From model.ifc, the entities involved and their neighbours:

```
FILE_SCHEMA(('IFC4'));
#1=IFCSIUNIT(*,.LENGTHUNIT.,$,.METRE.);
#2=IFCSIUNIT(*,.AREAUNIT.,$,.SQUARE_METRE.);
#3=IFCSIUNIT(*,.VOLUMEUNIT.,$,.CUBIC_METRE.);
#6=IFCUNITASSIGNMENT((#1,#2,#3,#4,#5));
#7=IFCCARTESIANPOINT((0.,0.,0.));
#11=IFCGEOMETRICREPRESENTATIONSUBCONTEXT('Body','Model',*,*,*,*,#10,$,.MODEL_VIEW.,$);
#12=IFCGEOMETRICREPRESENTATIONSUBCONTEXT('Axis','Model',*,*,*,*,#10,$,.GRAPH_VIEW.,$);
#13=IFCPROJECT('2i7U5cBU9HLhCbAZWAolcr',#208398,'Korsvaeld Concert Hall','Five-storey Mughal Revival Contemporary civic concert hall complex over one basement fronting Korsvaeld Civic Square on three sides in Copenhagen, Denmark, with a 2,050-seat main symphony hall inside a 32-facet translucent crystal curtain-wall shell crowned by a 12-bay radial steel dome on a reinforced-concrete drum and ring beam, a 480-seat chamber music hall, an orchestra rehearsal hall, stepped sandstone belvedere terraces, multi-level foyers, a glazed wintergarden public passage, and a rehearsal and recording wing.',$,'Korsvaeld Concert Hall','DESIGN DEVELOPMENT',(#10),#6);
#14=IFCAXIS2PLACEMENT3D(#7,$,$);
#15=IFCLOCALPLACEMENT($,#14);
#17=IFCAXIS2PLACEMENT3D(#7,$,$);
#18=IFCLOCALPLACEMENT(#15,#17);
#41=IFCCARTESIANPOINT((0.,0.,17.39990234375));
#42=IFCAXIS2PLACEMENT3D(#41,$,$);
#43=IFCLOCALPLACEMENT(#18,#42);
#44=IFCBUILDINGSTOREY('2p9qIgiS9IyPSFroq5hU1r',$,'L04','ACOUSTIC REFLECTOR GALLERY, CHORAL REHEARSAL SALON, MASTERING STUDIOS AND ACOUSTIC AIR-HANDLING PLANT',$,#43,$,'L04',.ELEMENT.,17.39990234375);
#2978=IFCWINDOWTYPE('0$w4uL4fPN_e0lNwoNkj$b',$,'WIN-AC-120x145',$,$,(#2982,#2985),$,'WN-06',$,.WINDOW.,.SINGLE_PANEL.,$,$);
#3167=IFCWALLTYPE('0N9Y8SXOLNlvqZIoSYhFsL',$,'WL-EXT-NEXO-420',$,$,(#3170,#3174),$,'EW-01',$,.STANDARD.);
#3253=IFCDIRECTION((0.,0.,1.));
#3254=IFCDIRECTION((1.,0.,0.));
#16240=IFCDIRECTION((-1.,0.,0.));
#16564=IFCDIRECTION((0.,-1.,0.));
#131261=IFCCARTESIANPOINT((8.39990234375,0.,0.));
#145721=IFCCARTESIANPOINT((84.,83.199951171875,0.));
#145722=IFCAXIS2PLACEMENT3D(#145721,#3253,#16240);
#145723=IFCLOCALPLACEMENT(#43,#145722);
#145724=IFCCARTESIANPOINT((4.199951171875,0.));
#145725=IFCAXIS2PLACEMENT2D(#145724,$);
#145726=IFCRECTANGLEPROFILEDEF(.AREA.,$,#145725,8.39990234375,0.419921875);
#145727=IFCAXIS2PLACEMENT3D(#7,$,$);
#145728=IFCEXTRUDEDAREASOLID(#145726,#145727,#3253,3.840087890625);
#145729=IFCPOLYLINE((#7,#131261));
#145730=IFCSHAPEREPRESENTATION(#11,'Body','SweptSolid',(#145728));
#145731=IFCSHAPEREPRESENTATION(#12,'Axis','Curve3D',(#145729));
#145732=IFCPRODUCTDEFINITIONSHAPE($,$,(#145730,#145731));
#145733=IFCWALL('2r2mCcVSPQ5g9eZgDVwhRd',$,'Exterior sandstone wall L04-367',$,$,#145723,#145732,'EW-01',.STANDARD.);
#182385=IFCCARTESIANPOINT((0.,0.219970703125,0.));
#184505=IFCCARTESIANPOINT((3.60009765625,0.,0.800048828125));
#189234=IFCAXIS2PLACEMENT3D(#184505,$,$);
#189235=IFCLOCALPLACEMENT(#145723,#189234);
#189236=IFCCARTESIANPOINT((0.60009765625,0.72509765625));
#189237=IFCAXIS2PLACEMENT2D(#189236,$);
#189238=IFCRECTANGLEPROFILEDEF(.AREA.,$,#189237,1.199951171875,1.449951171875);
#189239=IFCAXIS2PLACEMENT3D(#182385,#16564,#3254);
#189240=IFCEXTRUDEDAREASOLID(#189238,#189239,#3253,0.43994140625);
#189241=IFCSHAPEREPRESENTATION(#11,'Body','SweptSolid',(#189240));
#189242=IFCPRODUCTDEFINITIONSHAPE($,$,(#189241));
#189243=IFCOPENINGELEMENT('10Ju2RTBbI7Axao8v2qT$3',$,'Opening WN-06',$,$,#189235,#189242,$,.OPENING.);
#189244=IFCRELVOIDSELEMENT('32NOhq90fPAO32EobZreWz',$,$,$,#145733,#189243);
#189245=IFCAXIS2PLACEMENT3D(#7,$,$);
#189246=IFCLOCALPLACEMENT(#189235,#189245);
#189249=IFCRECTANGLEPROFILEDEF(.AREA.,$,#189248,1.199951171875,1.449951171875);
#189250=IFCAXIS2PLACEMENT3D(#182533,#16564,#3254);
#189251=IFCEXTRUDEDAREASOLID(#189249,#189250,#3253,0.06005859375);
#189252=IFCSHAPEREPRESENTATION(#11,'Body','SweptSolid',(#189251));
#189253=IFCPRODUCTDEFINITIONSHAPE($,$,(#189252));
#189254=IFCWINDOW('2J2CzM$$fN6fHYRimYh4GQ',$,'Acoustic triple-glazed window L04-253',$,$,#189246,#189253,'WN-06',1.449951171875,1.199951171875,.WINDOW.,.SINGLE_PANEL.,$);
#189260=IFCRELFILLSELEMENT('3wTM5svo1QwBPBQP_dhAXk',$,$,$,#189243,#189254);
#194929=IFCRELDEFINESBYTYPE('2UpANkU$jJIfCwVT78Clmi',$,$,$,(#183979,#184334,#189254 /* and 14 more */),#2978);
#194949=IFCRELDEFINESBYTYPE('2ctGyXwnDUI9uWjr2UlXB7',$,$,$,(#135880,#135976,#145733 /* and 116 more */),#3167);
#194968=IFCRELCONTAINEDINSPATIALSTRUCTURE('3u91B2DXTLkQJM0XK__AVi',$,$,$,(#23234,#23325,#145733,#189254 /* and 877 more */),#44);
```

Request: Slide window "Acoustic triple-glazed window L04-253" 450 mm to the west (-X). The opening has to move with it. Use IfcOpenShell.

```python
import ifcopenshell
import ifcopenshell.api.geometry
import ifcopenshell.util.placement
import ifcopenshell.util.unit

model = ifcopenshell.open("model.ifc")
unit_scale = ifcopenshell.util.unit.calculate_unit_scale(model)

window = model.by_id(189254)
opening = window.FillsVoids[0].RelatingOpeningElement
wall = opening.VoidsElements[0].RelatingBuildingElement

wall_matrix = ifcopenshell.util.placement.get_local_placement(wall.ObjectPlacement)
shift = wall_matrix[:3, 0] * 0.45 / unit_scale
before = ifcopenshell.util.placement.get_local_placement(window.ObjectPlacement)[:3, 3].copy()

# The window is placed relative to its opening, so it follows when the opening moves.
matrix = ifcopenshell.util.placement.get_local_placement(opening.ObjectPlacement)
matrix[:3, 3] += shift
ifcopenshell.api.geometry.edit_object_placement(
    model, product=opening, matrix=matrix, is_si=False, should_transform_children=True
)

after = ifcopenshell.util.placement.get_local_placement(window.ObjectPlacement)[:3, 3]
print("window moved by", (after - before).round(3) + 0.0)

model.write("model_v2.ifc")
```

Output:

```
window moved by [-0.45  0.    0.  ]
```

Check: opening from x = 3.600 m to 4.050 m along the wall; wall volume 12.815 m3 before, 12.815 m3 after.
